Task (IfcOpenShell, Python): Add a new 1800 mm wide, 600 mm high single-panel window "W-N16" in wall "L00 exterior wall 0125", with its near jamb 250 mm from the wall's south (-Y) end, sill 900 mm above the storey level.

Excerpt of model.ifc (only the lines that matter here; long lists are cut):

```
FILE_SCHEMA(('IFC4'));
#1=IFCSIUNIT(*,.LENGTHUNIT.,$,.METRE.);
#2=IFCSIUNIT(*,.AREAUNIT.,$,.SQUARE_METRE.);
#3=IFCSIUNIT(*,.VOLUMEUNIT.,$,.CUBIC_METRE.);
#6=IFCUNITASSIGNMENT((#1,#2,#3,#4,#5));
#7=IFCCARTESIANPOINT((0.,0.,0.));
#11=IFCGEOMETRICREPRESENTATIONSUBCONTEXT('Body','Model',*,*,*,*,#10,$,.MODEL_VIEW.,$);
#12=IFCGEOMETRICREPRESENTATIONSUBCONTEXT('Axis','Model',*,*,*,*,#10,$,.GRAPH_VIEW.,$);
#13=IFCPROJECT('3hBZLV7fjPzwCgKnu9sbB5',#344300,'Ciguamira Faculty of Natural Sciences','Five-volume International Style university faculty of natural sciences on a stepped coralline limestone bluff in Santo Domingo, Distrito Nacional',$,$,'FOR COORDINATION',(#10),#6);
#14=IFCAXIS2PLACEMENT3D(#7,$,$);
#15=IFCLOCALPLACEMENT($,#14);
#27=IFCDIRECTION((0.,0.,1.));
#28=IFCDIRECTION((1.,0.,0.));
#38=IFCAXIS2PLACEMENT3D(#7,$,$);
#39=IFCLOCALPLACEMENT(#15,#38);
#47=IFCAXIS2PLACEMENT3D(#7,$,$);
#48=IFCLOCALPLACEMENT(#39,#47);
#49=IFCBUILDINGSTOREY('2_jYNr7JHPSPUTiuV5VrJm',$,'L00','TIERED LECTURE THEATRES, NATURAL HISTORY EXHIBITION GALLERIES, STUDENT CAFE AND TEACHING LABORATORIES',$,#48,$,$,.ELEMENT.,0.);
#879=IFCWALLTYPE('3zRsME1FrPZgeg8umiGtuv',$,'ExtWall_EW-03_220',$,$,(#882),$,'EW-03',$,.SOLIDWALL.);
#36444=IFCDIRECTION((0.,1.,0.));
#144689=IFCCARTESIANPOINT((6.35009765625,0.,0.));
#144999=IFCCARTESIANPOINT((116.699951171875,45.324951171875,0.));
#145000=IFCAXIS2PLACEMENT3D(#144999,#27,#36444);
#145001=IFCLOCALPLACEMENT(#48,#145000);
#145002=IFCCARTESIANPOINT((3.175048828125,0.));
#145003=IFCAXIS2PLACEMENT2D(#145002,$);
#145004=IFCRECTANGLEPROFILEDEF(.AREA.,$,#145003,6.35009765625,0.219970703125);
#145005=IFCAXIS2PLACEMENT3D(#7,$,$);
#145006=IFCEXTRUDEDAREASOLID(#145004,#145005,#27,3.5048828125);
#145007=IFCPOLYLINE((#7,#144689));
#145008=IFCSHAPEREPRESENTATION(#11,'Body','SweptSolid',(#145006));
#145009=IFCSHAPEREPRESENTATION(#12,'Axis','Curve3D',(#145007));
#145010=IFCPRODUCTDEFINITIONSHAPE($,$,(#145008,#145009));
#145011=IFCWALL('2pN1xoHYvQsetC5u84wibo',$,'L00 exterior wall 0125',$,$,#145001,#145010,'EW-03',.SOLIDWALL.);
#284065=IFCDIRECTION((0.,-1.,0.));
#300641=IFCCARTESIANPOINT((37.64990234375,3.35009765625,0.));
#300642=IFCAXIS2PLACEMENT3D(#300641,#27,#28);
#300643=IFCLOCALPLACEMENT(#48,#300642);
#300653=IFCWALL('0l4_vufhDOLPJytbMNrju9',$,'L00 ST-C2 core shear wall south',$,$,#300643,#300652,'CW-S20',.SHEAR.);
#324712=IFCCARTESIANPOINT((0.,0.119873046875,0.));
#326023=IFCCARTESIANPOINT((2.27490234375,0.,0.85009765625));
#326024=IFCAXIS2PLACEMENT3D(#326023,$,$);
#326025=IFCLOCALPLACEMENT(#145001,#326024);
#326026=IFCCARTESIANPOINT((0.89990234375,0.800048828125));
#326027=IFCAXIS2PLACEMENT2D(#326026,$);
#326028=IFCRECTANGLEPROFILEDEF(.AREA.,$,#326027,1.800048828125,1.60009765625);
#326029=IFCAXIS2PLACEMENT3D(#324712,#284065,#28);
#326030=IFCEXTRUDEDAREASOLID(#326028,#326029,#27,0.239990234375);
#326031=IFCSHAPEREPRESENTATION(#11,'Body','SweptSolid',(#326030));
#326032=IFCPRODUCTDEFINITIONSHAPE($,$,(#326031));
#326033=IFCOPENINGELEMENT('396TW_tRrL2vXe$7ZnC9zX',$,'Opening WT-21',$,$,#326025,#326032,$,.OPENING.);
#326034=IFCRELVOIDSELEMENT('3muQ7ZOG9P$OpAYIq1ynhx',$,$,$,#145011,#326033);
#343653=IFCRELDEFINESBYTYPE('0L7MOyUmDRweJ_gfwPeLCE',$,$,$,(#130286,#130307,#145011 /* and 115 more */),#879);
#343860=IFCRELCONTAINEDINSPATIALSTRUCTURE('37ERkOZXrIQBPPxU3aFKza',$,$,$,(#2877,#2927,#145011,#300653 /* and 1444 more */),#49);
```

```python
import numpy as np
import ifcopenshell
import ifcopenshell.api.feature
import ifcopenshell.api.geometry
import ifcopenshell.api.root
import ifcopenshell.api.spatial
import ifcopenshell.geom
import ifcopenshell.util.element
import ifcopenshell.util.placement
import ifcopenshell.util.representation
import ifcopenshell.util.shape
import ifcopenshell.util.unit

model = ifcopenshell.open("model.ifc")
unit_scale = ifcopenshell.util.unit.calculate_unit_scale(model)
settings = ifcopenshell.geom.settings()


def volume(element):
    """Net volume in cubic metres, openings subtracted."""
    shape = ifcopenshell.geom.create_shape(settings, element)
    return ifcopenshell.util.shape.get_volume(shape.geometry)


wall = model.by_guid("2pN1xoHYvQsetC5u84wibo")
storey = ifcopenshell.util.element.get_container(wall, ifc_class="IfcBuildingStorey")
context = ifcopenshell.util.representation.get_context(model, "Model", "Body", "MODEL_VIEW")
before = volume(wall)

width, height, from_end, sill = 1.8, 0.6, 0.25, 0.9  # metres

# The wall runs along its own X axis, and the end named is its -X end.
wall_shape = ifcopenshell.geom.create_shape(settings, wall)
x, y, z = ifcopenshell.util.shape.get_vertices(wall_shape.geometry).T
start = x.min() + from_end
face, thickness = float(y.min()), float(y.max() - y.min())
wall_matrix = ifcopenshell.util.placement.get_local_placement(wall.ObjectPlacement)
level = ifcopenshell.util.placement.get_local_placement(storey.ObjectPlacement)[2, 3]


def in_wall(x, y):
    """Placement at x, y metres in the wall's axes, at sill height."""
    matrix = wall_matrix.copy()
    matrix[:, 3] = wall_matrix @ np.array([x / unit_scale, y / unit_scale, 0.0, 1.0])
    matrix[2, 3] = level + sill / unit_scale
    return matrix


# Opening: a box that overshoots both wall faces by 50 mm.
opening = ifcopenshell.api.root.create_entity(model, ifc_class="IfcOpeningElement", predefined_type="OPENING")
box = ifcopenshell.api.geometry.add_wall_representation(
    model, context=context, length=width, height=height, thickness=thickness + 0.1
)
ifcopenshell.api.geometry.assign_representation(model, product=opening, representation=box)
ifcopenshell.api.geometry.edit_object_placement(model, product=opening, matrix=in_wall(start, face - 0.05), is_si=False)
ifcopenshell.api.feature.add_feature(model, feature=opening, element=wall)

window = ifcopenshell.api.root.create_entity(model, ifc_class="IfcWindow", name="W-N16", predefined_type="WINDOW")
window.OverallWidth, window.OverallHeight = width / unit_scale, height / unit_scale
window.PartitioningType = "SINGLE_PANEL"
body = ifcopenshell.api.geometry.add_window_representation(
    model,
    context=context,
    overall_width=window.OverallWidth,
    overall_height=window.OverallHeight,
    partition_type="SINGLE_PANEL",
)
ifcopenshell.api.geometry.assign_representation(model, product=window, representation=body)
ifcopenshell.api.spatial.assign_container(model, products=[window], relating_structure=storey)
ifcopenshell.api.feature.add_filling(model, opening=opening, element=window)

# Centre the window in the wall's thickness.
ifcopenshell.api.geometry.edit_object_placement(model, product=window, matrix=in_wall(start, face), is_si=False)
window_shape = ifcopenshell.geom.create_shape(settings, window)
depth = ifcopenshell.util.shape.get_vertices(window_shape.geometry)[:, 1]
offset = face + thickness / 2 - (depth.min() + depth.max()) / 2
ifcopenshell.api.geometry.edit_object_placement(model, product=window, matrix=in_wall(start, offset), is_si=False)

after = volume(wall)

print(f"wall volume {before:.3f} -> {after:.3f} m3")

model.write("model_v2.ifc")
```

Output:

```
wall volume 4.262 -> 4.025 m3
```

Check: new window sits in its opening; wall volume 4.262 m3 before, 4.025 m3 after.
